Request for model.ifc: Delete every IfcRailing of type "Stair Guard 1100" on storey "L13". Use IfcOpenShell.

First a look at what the model holds.

```python
import ifcopenshell
import ifcopenshell.util.element

model = ifcopenshell.open("model.ifc")
print(model.schema)
storey = next(s for s in model.by_type("IfcBuildingStorey") if s.Name == "L13")
railings = [e for e in ifcopenshell.util.element.get_decomposition(storey) if e.is_a("IfcRailing")]
seen = {}
for e in railings:
    element_type = ifcopenshell.util.element.get_type(e)
    name = element_type.Name if element_type not in (None, e) else None
    seen[name] = seen.get(name, 0) + 1
for name, count in sorted(seen.items(), key=str):
    print(count, "x", name)
```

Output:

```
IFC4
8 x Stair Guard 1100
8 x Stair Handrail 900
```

```python
import ifcopenshell
import ifcopenshell.api.root
import ifcopenshell.util.element

model = ifcopenshell.open("model.ifc")

storey = next(s for s in model.by_type("IfcBuildingStorey") if s.Name == "L13")
railings = [e for e in ifcopenshell.util.element.get_decomposition(storey) if e.is_a("IfcRailing")]
targets = [e for e in railings if (t := ifcopenshell.util.element.get_type(e)) not in (None, e) and t.Name == "Stair Guard 1100"]

for e in targets:
    ifcopenshell.api.root.remove_product(model, product=e)
print(len(targets), "removed")

model.write("model_v2.ifc")
```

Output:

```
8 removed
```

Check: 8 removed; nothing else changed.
